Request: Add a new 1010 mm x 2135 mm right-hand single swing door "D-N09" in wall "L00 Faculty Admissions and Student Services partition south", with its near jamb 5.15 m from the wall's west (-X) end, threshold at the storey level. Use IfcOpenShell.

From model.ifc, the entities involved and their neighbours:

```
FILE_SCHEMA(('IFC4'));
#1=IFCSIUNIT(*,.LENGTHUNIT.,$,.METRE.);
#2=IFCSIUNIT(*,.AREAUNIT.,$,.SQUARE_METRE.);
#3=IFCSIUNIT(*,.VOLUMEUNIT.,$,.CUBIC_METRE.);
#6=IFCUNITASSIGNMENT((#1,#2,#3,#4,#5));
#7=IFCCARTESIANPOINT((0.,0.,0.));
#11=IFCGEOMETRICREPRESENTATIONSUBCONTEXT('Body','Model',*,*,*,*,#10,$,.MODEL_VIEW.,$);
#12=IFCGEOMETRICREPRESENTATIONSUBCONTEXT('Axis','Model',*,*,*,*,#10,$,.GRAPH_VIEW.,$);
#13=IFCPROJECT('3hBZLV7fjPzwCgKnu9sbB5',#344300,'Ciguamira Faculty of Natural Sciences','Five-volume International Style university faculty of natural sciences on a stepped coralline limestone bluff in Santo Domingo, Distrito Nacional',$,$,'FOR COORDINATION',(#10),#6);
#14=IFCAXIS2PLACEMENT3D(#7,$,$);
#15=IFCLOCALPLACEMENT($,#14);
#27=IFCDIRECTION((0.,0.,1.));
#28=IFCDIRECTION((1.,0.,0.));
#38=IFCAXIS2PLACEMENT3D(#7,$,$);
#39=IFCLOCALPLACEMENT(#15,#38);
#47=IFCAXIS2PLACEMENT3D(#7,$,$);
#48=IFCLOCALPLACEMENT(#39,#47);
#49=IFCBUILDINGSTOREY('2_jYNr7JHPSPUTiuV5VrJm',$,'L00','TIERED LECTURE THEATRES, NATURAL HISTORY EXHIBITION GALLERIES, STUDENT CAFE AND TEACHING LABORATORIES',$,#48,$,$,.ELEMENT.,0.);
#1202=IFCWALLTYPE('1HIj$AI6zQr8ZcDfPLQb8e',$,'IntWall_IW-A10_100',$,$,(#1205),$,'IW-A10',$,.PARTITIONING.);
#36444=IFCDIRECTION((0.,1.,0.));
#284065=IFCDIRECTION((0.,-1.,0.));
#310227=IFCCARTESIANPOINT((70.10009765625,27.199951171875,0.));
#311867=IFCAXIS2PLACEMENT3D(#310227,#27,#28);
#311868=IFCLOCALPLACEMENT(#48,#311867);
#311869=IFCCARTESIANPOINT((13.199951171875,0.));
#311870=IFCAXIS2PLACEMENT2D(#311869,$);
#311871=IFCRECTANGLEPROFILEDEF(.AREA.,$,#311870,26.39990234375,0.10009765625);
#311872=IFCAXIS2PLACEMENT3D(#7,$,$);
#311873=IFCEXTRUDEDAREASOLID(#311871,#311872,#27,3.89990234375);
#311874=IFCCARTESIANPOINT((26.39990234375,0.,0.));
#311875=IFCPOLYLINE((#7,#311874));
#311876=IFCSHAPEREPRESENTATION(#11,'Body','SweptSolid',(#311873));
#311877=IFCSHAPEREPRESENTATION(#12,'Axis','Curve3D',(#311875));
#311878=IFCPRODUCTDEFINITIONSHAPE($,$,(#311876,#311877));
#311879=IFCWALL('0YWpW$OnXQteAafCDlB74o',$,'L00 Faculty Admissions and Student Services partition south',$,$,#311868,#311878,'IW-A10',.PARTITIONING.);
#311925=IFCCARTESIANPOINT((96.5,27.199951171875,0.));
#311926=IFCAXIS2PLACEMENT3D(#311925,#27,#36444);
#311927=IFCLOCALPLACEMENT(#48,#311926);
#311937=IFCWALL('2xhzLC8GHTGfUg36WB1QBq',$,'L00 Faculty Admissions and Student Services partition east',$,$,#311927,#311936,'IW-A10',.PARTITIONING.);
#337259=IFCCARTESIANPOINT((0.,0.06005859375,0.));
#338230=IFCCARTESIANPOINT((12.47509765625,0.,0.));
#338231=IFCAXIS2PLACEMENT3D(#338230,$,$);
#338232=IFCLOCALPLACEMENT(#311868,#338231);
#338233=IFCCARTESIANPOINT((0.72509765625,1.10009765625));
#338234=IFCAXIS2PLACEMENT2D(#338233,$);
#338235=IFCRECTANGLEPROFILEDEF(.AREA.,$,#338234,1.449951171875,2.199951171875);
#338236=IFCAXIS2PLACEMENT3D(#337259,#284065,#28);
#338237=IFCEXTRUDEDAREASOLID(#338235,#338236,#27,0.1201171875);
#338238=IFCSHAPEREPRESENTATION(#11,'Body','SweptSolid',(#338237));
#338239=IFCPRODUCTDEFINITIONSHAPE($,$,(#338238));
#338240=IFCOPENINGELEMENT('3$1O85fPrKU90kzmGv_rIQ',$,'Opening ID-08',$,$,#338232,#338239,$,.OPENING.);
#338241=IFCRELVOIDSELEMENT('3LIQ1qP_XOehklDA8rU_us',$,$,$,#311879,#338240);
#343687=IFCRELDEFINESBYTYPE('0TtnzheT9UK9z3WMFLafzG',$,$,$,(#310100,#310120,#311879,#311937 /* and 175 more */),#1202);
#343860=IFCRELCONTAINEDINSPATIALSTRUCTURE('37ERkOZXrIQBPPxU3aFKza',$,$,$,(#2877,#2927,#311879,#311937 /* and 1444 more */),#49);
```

```python
import numpy as np
import ifcopenshell
import ifcopenshell.api.feature
import ifcopenshell.api.geometry
import ifcopenshell.api.root
import ifcopenshell.api.spatial
import ifcopenshell.geom
import ifcopenshell.util.element
import ifcopenshell.util.placement
import ifcopenshell.util.representation
import ifcopenshell.util.shape
import ifcopenshell.util.unit

model = ifcopenshell.open("model.ifc")
unit_scale = ifcopenshell.util.unit.calculate_unit_scale(model)
settings = ifcopenshell.geom.settings()


def volume(element):
    """Net volume in cubic metres, openings subtracted."""
    shape = ifcopenshell.geom.create_shape(settings, element)
    return ifcopenshell.util.shape.get_volume(shape.geometry)


wall = model.by_guid("0YWpW$OnXQteAafCDlB74o")
storey = ifcopenshell.util.element.get_container(wall, ifc_class="IfcBuildingStorey")
context = ifcopenshell.util.representation.get_context(model, "Model", "Body", "MODEL_VIEW")
before = volume(wall)

width, height, from_end, sill = 1.01, 2.135, 5.15, 0.0  # metres

# The wall runs along its own X axis, and the end named is its -X end.
wall_shape = ifcopenshell.geom.create_shape(settings, wall)
x, y, z = ifcopenshell.util.shape.get_vertices(wall_shape.geometry).T
start = x.min() + from_end
face, thickness = float(y.min()), float(y.max() - y.min())
wall_matrix = ifcopenshell.util.placement.get_local_placement(wall.ObjectPlacement)
level = ifcopenshell.util.placement.get_local_placement(storey.ObjectPlacement)[2, 3]


def in_wall(x, y):
    """Placement at x, y metres in the wall's axes, at sill height."""
    matrix = wall_matrix.copy()
    matrix[:, 3] = wall_matrix @ np.array([x / unit_scale, y / unit_scale, 0.0, 1.0])
    matrix[2, 3] = level + sill / unit_scale
    return matrix


# Opening: a box that overshoots both wall faces by 50 mm.
opening = ifcopenshell.api.root.create_entity(model, ifc_class="IfcOpeningElement", predefined_type="OPENING")
box = ifcopenshell.api.geometry.add_wall_representation(
    model, context=context, length=width, height=height, thickness=thickness + 0.1
)
ifcopenshell.api.geometry.assign_representation(model, product=opening, representation=box)
ifcopenshell.api.geometry.edit_object_placement(model, product=opening, matrix=in_wall(start, face - 0.05), is_si=False)
ifcopenshell.api.feature.add_feature(model, feature=opening, element=wall)

door = ifcopenshell.api.root.create_entity(model, ifc_class="IfcDoor", name="D-N09", predefined_type="DOOR")
door.OverallWidth, door.OverallHeight = width / unit_scale, height / unit_scale
door.OperationType = "SINGLE_SWING_RIGHT"
body = ifcopenshell.api.geometry.add_door_representation(
    model,
    context=context,
    overall_width=door.OverallWidth,
    overall_height=door.OverallHeight,
    operation_type="SINGLE_SWING_RIGHT",
    lining_properties={"LiningDepth": thickness / unit_scale, "ThresholdDepth": thickness / unit_scale},
)
ifcopenshell.api.geometry.assign_representation(model, product=door, representation=body)
ifcopenshell.api.spatial.assign_container(model, products=[door], relating_structure=storey)
ifcopenshell.api.feature.add_filling(model, opening=opening, element=door)

# The lining spans the wall, so the door starts at the wall face.
ifcopenshell.api.geometry.edit_object_placement(model, product=door, matrix=in_wall(start, face), is_si=False)

after = volume(wall)

print(f"wall volume {before:.3f} -> {after:.3f} m3")

model.write("model_rev.ifc")
```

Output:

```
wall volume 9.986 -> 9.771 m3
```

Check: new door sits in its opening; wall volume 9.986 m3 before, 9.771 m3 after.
